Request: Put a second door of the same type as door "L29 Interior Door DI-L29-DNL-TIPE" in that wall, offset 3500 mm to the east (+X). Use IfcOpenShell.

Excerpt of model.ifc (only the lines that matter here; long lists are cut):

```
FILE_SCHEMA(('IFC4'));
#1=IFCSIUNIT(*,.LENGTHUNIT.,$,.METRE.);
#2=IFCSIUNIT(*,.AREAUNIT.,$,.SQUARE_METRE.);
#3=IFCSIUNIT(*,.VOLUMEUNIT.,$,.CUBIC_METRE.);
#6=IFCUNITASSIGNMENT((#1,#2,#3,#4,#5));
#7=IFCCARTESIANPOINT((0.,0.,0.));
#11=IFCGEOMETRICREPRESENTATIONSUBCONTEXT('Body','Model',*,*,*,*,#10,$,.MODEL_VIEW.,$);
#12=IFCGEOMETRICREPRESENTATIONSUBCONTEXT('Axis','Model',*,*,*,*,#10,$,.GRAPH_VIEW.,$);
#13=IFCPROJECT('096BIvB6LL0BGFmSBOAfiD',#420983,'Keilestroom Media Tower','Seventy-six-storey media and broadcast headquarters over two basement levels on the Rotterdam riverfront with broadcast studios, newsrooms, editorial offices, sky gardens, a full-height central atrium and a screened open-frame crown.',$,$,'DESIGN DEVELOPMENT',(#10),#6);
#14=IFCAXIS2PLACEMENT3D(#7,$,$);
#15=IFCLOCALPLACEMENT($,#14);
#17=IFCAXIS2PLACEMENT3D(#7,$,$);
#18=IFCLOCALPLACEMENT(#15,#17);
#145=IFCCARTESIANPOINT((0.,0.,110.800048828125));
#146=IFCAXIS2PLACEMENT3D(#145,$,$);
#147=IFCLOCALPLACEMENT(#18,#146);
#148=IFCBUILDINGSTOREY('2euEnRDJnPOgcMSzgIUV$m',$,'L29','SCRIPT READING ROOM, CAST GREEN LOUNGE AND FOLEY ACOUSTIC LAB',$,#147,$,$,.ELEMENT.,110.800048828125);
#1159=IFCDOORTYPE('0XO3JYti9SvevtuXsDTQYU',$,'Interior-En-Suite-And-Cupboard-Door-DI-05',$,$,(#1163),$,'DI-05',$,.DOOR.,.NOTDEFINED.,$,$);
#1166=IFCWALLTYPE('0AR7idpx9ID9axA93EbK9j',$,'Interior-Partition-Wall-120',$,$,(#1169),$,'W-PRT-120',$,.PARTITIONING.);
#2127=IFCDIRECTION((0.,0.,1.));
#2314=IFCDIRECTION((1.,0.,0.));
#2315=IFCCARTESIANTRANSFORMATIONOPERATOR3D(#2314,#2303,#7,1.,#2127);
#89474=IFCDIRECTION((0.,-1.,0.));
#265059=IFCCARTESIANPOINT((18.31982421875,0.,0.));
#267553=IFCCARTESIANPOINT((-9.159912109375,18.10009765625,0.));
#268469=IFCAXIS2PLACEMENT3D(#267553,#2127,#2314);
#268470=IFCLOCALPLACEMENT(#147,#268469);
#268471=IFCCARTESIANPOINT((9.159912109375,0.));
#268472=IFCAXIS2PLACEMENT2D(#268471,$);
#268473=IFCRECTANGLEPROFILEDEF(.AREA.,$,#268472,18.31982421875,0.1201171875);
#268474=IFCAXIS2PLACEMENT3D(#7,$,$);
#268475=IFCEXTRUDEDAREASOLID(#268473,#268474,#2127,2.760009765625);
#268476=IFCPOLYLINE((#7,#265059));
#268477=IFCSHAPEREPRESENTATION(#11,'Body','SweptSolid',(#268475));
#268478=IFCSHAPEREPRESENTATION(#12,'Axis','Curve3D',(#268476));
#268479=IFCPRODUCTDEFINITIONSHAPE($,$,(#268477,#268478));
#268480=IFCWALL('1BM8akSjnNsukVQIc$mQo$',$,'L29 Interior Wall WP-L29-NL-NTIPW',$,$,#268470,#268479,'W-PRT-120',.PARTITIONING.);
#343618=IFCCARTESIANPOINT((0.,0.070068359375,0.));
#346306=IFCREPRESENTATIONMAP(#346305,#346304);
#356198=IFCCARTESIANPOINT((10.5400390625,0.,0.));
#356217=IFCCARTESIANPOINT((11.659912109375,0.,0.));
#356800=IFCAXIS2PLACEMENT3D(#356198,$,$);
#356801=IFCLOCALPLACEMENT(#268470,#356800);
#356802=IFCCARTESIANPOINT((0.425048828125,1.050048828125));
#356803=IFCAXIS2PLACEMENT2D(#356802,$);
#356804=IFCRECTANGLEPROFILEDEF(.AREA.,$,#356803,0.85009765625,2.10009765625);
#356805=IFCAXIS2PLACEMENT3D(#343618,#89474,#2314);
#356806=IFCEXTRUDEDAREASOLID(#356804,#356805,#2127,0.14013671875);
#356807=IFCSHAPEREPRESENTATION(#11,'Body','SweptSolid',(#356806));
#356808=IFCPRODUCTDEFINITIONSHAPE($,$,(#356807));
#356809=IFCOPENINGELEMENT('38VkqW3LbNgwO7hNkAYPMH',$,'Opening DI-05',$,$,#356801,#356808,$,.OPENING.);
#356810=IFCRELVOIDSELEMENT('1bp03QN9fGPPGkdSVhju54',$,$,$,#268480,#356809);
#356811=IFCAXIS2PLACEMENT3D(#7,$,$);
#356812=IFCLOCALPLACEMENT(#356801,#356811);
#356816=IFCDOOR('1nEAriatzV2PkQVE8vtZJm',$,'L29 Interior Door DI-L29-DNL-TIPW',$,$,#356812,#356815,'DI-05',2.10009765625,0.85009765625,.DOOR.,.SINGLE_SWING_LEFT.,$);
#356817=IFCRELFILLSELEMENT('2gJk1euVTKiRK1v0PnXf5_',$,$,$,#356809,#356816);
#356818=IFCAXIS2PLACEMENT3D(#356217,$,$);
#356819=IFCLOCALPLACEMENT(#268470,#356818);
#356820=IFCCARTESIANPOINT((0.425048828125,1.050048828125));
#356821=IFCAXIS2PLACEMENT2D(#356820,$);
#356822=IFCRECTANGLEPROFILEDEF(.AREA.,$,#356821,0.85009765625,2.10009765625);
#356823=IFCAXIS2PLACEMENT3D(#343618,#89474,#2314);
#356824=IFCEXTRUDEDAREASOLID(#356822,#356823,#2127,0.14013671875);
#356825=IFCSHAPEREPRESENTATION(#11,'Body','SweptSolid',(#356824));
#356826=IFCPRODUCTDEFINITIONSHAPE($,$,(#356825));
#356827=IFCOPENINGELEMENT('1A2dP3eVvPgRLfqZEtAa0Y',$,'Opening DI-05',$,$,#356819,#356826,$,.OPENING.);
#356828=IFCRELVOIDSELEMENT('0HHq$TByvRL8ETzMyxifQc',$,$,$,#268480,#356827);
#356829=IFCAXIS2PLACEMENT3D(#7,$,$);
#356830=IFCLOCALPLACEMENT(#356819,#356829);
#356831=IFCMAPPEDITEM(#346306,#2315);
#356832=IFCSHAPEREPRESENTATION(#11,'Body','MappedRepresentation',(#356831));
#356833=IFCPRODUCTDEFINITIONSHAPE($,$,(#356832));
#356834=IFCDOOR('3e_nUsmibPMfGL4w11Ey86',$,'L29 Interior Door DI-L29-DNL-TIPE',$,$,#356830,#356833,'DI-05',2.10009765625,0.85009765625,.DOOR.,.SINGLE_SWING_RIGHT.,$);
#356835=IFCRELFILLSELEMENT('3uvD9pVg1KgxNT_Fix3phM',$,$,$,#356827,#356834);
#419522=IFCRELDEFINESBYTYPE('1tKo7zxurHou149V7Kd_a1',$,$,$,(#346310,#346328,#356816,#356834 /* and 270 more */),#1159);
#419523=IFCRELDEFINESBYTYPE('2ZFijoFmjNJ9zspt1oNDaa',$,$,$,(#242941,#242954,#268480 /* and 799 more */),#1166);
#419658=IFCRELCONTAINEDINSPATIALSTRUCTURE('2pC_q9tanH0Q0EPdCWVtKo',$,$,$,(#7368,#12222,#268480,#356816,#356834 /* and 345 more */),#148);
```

```python
import ifcopenshell
import ifcopenshell.api.feature
import ifcopenshell.api.geometry
import ifcopenshell.api.root
import ifcopenshell.geom
import ifcopenshell.util.element
import ifcopenshell.util.placement
import ifcopenshell.util.shape
import ifcopenshell.util.unit

model = ifcopenshell.open("model.ifc")
unit_scale = ifcopenshell.util.unit.calculate_unit_scale(model)
settings = ifcopenshell.geom.settings()


def volume(element):
    """Net volume in cubic metres, openings subtracted."""
    shape = ifcopenshell.geom.create_shape(settings, element)
    return ifcopenshell.util.shape.get_volume(shape.geometry)


door = model.by_guid("3e_nUsmibPMfGL4w11Ey86")
opening = door.FillsVoids[0].RelatingOpeningElement
wall = opening.VoidsElements[0].RelatingBuildingElement
before = volume(wall)
shift = ifcopenshell.util.placement.get_local_placement(wall.ObjectPlacement)[:3, 0] * 3.5 / unit_scale

# copy_class copies the void relationship, type, container and properties, but no geometry.
new_opening = ifcopenshell.api.root.copy_class(model, product=opening)
new_opening.Representation = ifcopenshell.util.element.copy_deep(
    model, opening.Representation, exclude=["IfcGeometricRepresentationContext", "IfcRepresentationMap"]
)
new_door = ifcopenshell.api.root.copy_class(model, product=door)
new_door.Representation = ifcopenshell.util.element.copy_deep(
    model, door.Representation, exclude=["IfcGeometricRepresentationContext", "IfcRepresentationMap"]
)
new_door.Tag = None
ifcopenshell.api.feature.add_filling(model, opening=new_opening, element=new_door)

for old, new in ((opening, new_opening), (door, new_door)):
    matrix = ifcopenshell.util.placement.get_local_placement(old.ObjectPlacement)
    matrix[:3, 3] += shift
    ifcopenshell.api.geometry.edit_object_placement(model, product=new, matrix=matrix, is_si=False)

after = volume(wall)

print(f"wall volume {before:.3f} -> {after:.3f} m3")

model.write("model-out.ifc")
```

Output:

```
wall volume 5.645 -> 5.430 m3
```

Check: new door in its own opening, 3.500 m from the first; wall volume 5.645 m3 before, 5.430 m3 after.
